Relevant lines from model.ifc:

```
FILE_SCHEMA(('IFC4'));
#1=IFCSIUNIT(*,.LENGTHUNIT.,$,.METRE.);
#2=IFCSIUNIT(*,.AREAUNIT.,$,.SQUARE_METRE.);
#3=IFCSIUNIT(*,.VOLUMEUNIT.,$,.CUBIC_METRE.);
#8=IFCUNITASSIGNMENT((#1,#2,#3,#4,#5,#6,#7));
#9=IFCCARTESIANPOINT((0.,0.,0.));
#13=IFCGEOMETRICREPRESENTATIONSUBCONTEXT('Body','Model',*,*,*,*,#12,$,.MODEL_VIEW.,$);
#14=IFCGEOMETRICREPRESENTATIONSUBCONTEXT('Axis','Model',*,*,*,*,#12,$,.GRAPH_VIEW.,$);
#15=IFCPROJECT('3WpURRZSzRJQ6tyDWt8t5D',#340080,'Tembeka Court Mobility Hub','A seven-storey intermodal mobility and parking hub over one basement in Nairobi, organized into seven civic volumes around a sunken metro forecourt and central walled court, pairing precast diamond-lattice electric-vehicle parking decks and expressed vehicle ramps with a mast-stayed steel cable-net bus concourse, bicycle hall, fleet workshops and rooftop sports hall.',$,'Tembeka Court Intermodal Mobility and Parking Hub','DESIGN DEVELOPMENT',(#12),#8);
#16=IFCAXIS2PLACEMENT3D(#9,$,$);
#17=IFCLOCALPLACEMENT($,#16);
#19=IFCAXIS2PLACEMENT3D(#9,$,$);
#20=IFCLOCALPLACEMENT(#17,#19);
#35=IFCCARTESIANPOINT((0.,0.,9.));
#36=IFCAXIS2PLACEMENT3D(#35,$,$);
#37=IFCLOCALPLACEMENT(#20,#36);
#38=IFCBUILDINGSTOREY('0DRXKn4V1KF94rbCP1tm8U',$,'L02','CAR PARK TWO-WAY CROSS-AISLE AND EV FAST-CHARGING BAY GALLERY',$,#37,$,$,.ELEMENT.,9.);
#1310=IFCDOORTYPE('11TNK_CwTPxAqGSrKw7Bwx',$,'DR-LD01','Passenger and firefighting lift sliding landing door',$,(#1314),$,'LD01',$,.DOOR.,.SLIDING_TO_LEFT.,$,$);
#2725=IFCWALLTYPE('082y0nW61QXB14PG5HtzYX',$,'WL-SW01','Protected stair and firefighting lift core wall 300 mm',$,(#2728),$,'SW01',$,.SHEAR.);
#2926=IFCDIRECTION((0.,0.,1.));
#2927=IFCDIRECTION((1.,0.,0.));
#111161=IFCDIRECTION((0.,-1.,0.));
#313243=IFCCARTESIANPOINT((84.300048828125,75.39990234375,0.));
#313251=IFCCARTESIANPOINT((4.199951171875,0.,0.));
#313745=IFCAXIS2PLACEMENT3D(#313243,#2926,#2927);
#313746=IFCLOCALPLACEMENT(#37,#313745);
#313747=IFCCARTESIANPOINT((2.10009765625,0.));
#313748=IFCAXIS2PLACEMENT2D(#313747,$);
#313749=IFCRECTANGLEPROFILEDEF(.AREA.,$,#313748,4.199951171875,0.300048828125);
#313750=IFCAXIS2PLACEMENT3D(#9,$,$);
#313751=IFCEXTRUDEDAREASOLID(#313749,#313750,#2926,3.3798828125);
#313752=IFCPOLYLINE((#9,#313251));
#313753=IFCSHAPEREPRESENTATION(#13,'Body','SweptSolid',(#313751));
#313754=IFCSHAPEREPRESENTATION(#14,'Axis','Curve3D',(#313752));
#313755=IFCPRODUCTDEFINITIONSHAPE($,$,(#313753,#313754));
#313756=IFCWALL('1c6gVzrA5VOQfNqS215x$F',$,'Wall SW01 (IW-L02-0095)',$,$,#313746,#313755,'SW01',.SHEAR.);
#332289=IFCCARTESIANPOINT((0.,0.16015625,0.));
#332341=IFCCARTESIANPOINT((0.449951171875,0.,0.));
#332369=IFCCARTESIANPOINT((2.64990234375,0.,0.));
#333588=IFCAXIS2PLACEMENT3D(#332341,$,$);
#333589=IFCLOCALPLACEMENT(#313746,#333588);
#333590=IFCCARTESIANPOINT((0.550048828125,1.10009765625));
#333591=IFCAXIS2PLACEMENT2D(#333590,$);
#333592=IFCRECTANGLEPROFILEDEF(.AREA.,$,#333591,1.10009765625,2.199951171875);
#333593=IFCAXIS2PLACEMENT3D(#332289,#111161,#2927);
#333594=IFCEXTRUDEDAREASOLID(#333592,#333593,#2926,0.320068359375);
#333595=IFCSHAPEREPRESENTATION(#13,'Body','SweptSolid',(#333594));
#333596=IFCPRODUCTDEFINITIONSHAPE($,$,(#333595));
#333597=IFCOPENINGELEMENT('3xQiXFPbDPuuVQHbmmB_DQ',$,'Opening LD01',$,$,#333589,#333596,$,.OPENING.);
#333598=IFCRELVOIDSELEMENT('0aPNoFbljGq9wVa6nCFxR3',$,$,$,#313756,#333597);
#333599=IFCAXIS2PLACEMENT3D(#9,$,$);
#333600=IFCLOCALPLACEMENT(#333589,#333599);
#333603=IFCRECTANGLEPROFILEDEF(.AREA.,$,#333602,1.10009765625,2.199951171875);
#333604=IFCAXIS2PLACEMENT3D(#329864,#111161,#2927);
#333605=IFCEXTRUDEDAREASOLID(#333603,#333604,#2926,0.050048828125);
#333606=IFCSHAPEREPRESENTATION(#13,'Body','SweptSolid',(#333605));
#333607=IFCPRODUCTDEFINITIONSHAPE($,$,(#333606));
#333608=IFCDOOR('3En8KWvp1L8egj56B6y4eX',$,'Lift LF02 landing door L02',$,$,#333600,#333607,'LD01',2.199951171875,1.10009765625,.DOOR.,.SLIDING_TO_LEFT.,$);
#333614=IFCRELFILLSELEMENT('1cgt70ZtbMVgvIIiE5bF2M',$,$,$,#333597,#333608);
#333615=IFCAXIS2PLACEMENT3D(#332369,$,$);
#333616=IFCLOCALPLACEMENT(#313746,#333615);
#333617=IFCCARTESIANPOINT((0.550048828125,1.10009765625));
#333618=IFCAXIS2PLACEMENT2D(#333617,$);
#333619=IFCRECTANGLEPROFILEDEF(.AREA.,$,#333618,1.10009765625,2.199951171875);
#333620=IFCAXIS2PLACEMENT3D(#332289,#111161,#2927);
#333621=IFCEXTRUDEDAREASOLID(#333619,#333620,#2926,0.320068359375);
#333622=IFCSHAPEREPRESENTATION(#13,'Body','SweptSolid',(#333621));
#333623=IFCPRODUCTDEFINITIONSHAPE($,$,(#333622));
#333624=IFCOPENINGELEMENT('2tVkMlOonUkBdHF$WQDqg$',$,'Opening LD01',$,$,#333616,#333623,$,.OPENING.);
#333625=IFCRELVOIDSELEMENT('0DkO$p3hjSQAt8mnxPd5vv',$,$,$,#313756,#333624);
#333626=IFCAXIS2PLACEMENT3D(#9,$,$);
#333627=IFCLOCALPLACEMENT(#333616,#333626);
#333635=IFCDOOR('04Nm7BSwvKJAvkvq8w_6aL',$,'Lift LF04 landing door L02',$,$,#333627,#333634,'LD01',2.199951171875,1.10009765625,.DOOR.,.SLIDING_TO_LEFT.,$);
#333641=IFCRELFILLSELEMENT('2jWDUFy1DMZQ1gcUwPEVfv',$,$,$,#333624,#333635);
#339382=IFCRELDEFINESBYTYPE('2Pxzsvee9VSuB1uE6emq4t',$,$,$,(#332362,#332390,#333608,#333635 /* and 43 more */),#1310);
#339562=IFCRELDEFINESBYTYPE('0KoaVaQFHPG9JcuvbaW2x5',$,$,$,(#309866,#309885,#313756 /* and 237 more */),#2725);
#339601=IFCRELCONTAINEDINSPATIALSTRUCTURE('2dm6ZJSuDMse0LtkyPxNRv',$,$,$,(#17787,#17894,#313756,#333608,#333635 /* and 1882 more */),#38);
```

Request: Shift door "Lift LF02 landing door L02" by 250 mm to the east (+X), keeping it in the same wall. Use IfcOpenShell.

```python
import ifcopenshell
import ifcopenshell.api.geometry
import ifcopenshell.util.placement

model = ifcopenshell.open("model.ifc")

door = model.by_guid("3En8KWvp1L8egj56B6y4eX")
opening = door.FillsVoids[0].RelatingOpeningElement
wall = opening.VoidsElements[0].RelatingBuildingElement

wall_matrix = ifcopenshell.util.placement.get_local_placement(wall.ObjectPlacement)
shift = wall_matrix[:3, 0] * 0.25
before = ifcopenshell.util.placement.get_local_placement(door.ObjectPlacement)[:3, 3].copy()

# The door is placed relative to its opening, so it follows when the opening moves.
matrix = ifcopenshell.util.placement.get_local_placement(opening.ObjectPlacement)
matrix[:3, 3] += shift
ifcopenshell.api.geometry.edit_object_placement(
    model, product=opening, matrix=matrix, is_si=False, should_transform_children=True
)

after = ifcopenshell.util.placement.get_local_placement(door.ObjectPlacement)[:3, 3]
print("door moved by", (after - before).round(3) + 0.0)

model.write("model_v2.ifc")
```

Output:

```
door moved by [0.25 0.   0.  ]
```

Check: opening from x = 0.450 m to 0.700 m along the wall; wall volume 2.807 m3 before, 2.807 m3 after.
